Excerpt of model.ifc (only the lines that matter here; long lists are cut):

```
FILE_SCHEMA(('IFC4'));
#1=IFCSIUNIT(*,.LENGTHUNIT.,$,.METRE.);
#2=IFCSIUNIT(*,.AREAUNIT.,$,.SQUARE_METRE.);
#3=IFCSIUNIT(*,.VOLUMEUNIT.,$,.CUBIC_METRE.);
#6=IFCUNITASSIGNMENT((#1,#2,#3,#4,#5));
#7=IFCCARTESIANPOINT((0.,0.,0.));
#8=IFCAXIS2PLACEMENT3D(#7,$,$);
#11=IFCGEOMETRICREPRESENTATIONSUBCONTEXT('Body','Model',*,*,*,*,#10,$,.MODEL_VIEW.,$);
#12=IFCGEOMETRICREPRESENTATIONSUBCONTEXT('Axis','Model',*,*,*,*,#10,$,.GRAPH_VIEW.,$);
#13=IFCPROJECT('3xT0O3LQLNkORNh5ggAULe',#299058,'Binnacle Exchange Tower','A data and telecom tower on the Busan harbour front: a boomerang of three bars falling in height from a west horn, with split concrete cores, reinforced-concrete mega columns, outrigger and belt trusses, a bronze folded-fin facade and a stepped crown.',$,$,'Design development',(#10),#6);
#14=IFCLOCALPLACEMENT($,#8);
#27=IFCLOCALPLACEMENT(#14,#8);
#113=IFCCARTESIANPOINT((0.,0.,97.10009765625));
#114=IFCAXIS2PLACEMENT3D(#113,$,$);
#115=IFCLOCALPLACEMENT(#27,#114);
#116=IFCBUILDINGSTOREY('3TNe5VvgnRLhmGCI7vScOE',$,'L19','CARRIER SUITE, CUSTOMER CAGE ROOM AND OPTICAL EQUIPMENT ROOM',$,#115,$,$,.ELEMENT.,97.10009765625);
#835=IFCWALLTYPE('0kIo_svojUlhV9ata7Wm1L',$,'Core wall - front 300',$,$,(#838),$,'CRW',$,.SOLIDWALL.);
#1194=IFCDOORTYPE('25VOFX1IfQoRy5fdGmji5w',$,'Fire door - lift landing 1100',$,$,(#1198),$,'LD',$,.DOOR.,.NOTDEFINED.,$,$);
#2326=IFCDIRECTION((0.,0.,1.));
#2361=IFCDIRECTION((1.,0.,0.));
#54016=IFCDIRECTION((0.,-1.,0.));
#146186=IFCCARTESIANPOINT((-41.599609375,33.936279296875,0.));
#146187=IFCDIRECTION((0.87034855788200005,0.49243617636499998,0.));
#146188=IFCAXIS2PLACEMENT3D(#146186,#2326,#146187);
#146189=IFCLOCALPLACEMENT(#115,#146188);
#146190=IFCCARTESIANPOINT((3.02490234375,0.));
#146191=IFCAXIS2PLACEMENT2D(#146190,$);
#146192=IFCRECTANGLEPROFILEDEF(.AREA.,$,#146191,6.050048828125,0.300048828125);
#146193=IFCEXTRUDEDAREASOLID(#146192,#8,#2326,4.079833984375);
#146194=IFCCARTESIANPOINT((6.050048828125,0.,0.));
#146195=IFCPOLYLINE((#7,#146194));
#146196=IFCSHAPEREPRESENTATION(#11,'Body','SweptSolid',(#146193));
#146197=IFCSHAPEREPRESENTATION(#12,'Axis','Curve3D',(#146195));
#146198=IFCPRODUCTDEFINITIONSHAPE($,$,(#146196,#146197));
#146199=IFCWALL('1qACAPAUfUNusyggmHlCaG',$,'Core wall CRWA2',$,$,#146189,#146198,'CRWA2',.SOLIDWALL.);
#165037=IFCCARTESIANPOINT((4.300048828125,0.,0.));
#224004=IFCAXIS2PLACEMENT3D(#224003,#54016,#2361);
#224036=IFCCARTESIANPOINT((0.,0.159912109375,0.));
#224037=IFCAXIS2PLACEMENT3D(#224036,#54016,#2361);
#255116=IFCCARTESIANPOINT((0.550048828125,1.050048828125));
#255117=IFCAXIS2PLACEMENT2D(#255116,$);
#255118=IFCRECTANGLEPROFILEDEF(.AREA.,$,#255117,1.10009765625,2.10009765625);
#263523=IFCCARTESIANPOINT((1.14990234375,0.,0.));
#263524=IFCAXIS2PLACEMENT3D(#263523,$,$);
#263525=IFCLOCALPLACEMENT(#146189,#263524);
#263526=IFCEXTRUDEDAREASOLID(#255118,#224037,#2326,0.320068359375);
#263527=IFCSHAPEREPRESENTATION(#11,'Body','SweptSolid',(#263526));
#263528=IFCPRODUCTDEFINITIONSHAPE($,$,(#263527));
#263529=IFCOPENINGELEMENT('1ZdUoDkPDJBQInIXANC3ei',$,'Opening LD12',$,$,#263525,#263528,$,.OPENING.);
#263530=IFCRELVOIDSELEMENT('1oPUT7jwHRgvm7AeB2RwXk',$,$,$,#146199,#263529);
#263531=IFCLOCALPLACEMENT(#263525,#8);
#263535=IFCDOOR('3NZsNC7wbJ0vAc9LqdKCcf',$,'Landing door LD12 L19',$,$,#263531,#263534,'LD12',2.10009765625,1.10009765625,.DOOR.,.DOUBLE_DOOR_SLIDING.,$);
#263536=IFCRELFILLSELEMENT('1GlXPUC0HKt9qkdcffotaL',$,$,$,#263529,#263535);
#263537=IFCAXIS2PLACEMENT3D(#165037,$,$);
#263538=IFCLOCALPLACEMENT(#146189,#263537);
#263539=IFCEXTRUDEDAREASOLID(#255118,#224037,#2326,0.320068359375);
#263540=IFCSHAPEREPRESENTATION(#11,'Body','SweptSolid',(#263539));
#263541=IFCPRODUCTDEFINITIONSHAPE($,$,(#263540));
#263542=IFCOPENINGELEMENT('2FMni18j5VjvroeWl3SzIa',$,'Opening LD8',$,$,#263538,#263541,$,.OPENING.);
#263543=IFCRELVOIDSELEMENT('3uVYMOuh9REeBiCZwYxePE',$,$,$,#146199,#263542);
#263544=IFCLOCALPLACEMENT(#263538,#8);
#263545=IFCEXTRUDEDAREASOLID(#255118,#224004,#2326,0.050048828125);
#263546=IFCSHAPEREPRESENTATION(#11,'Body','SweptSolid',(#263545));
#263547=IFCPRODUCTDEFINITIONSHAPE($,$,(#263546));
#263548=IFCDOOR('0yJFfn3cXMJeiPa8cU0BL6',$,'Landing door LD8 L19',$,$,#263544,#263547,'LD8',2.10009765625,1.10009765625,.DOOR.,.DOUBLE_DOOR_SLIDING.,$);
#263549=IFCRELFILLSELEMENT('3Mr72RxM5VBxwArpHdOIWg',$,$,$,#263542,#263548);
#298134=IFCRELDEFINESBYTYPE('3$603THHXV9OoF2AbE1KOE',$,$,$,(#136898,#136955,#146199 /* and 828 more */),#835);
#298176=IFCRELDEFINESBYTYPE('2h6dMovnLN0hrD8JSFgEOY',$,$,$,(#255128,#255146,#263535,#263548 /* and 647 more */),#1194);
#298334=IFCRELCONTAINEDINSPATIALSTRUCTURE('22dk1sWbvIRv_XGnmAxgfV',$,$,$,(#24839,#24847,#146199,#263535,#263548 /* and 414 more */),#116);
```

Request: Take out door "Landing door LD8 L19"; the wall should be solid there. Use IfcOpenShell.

```python
import ifcopenshell
import ifcopenshell.api.feature
import ifcopenshell.api.root
import ifcopenshell.geom
import ifcopenshell.util.shape

model = ifcopenshell.open("model.ifc")
settings = ifcopenshell.geom.settings()


def volume(element):
    """Net volume in cubic metres, openings subtracted."""
    shape = ifcopenshell.geom.create_shape(settings, element)
    return ifcopenshell.util.shape.get_volume(shape.geometry)


door = model.by_guid("0yJFfn3cXMJeiPa8cU0BL6")
opening = door.FillsVoids[0].RelatingOpeningElement
wall = opening.VoidsElements[0].RelatingBuildingElement
before = volume(wall)

ifcopenshell.api.root.remove_product(model, product=door)
ifcopenshell.api.feature.remove_feature(model, feature=opening)

after = volume(wall)

print(f"wall volume {before:.3f} -> {after:.3f} m3")

model.write("model_v2.ifc")
```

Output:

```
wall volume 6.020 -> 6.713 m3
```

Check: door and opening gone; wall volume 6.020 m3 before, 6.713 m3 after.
